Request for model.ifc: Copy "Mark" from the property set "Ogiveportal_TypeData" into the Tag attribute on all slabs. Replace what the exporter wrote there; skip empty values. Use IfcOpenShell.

First a look at what the model holds.

```python
import ifcopenshell
import ifcopenshell.util.element

model = ifcopenshell.open("model.ifc")
print(model.schema)
slabs = model.by_type("IfcSlab")
print(len(slabs), "slabs")
for e in slabs[:8]:
    source = ifcopenshell.util.element.get_pset(e, "Ogiveportal_TypeData", "Mark")
    target = e.Tag
    print(e.id(), repr(source), repr(target), sep=" | ")
```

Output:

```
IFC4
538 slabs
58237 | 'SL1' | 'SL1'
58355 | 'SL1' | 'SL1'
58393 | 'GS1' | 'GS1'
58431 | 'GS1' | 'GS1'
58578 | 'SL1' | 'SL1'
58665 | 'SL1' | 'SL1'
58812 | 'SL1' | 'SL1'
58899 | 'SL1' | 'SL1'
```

```python
import ifcopenshell
import ifcopenshell.util.element

model = ifcopenshell.open("model.ifc")

count = 0
for e in model.by_type("IfcSlab"):
    value = ifcopenshell.util.element.get_pset(e, "Ogiveportal_TypeData", "Mark")
    current = e.Tag
    if not value or not value.strip() or current == value:
        continue
    e.Tag = value
    count += 1

print(count, "slabs updated")

model.write("model_updated.ifc")
```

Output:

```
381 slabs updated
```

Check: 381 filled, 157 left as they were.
